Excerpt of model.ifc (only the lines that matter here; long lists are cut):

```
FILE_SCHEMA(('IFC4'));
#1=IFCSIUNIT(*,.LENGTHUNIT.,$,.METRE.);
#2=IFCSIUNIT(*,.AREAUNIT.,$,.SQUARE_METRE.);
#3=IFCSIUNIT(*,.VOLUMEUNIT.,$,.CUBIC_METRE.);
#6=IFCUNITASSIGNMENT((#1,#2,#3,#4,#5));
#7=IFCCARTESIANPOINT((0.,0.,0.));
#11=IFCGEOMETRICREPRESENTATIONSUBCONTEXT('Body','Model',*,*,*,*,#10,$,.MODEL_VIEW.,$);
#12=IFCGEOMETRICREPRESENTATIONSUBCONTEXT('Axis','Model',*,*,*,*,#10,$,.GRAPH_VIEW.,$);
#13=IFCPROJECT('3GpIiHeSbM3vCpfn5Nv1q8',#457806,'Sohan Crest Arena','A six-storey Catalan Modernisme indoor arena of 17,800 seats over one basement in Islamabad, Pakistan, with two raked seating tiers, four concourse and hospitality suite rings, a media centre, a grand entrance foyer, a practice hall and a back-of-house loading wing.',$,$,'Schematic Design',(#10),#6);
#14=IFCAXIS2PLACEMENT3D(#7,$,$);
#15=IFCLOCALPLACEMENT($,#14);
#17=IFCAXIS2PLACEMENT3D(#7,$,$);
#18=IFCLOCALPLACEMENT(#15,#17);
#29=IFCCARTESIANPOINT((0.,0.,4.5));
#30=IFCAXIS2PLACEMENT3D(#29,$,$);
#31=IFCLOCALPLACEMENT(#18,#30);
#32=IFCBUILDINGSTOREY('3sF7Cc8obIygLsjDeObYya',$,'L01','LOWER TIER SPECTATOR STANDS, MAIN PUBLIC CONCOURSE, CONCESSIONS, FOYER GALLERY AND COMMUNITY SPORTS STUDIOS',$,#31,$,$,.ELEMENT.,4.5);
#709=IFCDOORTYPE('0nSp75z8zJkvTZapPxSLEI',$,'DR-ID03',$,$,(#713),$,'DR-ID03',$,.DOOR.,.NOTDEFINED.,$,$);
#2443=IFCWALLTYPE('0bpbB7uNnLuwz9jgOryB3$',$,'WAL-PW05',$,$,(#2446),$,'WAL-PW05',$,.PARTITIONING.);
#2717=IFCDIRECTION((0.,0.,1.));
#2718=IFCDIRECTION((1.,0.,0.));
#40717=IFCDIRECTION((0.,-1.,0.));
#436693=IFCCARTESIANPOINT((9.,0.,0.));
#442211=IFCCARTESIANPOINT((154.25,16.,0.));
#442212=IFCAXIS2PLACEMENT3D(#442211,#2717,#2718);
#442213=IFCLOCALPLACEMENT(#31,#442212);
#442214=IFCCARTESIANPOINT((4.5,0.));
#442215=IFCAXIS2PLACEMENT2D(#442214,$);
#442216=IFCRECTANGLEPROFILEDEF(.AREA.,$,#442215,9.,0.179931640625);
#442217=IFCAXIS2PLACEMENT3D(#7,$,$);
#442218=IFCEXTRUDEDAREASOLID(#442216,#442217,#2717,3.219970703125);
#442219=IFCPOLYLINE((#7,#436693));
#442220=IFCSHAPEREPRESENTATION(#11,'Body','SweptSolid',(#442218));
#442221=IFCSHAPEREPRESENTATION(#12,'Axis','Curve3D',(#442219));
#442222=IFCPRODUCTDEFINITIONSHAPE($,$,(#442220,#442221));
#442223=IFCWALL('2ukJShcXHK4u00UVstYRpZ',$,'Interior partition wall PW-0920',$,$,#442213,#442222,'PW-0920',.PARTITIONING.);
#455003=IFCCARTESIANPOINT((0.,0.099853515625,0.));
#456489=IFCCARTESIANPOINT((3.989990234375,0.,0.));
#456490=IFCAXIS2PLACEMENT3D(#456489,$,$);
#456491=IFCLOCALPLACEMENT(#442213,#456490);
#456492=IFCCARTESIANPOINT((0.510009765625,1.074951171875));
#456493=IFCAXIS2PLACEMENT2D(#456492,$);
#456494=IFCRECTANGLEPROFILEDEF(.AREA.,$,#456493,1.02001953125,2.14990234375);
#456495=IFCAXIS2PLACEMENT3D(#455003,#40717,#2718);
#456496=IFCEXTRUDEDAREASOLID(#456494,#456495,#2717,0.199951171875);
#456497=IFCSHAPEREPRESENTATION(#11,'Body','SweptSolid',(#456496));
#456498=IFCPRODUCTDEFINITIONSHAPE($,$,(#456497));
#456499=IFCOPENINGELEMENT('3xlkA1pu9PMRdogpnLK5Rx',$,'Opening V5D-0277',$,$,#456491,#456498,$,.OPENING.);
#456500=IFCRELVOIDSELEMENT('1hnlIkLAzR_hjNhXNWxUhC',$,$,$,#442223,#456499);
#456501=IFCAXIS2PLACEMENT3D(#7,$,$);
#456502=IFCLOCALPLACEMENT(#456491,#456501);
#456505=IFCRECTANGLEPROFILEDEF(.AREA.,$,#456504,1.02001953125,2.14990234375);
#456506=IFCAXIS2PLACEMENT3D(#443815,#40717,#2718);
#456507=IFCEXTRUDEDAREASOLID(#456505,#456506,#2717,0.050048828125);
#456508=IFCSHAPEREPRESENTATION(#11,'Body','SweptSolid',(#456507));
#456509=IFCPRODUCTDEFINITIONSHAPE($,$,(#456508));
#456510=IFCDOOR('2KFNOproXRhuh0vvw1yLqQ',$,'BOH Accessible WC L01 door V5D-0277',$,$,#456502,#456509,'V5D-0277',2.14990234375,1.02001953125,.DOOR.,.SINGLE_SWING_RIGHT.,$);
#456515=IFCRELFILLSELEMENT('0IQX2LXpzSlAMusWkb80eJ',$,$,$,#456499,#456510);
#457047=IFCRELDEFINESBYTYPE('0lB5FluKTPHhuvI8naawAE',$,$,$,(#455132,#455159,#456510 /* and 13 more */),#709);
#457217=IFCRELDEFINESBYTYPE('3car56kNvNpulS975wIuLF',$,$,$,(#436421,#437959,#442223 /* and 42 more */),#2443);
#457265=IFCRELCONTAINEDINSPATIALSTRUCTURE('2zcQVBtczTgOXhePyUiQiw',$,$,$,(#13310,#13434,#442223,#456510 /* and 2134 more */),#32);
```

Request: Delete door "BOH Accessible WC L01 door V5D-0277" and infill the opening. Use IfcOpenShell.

```python
import ifcopenshell
import ifcopenshell.api.feature
import ifcopenshell.api.root
import ifcopenshell.geom
import ifcopenshell.util.shape

model = ifcopenshell.open("model.ifc")
settings = ifcopenshell.geom.settings()


def volume(element):
    """Net volume in cubic metres, openings subtracted."""
    shape = ifcopenshell.geom.create_shape(settings, element)
    return ifcopenshell.util.shape.get_volume(shape.geometry)


door = model.by_id(456510)
opening = door.FillsVoids[0].RelatingOpeningElement
wall = opening.VoidsElements[0].RelatingBuildingElement
before = volume(wall)

ifcopenshell.api.root.remove_product(model, product=door)
ifcopenshell.api.feature.remove_feature(model, feature=opening)

after = volume(wall)

print(f"wall volume {before:.3f} -> {after:.3f} m3")

model.write("model_rev.ifc")
```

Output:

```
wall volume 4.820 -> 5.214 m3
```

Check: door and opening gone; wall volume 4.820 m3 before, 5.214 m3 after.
